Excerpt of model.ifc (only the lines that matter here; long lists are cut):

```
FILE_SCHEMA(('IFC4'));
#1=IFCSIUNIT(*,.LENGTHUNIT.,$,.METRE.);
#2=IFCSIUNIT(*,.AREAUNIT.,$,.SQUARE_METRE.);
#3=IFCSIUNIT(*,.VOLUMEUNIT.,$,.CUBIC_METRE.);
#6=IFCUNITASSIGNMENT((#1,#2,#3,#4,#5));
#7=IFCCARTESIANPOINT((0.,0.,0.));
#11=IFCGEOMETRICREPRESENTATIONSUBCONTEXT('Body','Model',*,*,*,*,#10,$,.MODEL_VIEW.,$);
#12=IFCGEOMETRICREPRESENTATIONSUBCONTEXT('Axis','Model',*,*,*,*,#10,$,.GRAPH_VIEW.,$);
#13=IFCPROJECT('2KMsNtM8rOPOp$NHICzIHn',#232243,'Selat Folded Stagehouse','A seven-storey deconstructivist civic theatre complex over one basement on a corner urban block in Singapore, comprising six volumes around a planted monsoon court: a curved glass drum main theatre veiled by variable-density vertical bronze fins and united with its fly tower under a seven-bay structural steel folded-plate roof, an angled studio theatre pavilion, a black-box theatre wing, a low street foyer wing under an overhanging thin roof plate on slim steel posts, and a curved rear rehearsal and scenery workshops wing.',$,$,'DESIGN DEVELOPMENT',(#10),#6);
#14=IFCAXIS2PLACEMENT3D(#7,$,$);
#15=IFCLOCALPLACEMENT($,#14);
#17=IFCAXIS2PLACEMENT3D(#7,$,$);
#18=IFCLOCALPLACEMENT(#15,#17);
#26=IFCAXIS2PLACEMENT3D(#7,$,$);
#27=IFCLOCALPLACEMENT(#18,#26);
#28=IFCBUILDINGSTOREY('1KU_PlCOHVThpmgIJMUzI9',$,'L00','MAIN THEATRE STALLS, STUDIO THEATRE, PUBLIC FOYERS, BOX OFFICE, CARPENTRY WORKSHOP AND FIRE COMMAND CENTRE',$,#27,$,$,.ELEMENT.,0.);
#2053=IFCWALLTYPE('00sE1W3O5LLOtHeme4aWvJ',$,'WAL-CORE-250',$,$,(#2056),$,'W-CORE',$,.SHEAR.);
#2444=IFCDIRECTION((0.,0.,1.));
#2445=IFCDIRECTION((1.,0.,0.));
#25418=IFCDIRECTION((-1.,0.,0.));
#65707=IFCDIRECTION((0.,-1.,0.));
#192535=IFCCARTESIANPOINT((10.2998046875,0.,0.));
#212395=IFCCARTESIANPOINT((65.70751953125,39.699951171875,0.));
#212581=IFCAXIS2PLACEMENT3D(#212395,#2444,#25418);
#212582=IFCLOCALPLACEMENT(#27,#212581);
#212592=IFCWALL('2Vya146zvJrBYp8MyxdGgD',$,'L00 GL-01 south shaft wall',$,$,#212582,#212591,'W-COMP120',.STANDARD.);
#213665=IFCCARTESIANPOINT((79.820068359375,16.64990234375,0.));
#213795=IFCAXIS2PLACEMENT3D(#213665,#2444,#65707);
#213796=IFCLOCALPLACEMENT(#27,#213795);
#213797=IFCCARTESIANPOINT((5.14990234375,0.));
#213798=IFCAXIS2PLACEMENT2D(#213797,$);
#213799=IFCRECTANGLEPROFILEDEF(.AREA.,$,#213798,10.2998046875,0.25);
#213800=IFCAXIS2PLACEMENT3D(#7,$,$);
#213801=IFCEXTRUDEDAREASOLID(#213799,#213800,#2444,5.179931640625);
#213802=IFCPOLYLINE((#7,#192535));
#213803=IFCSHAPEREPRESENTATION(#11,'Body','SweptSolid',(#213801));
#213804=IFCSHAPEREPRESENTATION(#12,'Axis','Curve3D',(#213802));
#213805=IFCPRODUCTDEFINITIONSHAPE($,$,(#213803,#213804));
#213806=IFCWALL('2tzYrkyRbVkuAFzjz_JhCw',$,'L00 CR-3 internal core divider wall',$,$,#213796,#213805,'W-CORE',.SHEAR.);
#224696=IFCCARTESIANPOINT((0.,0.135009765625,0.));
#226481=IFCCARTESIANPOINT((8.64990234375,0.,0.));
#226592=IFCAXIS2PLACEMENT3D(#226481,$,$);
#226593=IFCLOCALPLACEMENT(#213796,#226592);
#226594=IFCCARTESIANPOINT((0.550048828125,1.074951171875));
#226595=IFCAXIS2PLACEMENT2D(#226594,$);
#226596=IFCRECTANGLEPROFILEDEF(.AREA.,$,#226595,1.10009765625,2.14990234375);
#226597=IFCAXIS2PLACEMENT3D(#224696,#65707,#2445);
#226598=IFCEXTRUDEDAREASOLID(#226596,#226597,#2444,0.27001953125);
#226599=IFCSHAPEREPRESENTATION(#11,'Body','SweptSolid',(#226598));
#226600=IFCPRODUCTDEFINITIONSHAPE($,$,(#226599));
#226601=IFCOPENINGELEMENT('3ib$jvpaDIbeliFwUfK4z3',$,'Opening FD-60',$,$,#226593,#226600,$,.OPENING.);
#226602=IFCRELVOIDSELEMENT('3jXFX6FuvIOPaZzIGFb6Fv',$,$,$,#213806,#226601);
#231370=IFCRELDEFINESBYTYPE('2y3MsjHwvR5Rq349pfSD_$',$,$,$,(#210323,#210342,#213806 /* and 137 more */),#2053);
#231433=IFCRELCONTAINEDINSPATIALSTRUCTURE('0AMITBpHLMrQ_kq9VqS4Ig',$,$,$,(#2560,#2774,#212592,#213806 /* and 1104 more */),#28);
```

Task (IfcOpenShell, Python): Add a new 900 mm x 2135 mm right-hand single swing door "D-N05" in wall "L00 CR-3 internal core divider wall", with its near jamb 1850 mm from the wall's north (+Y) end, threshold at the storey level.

```python
import numpy as np
import ifcopenshell
import ifcopenshell.api.feature
import ifcopenshell.api.geometry
import ifcopenshell.api.root
import ifcopenshell.api.spatial
import ifcopenshell.geom
import ifcopenshell.util.element
import ifcopenshell.util.placement
import ifcopenshell.util.representation
import ifcopenshell.util.shape
import ifcopenshell.util.unit

model = ifcopenshell.open("model.ifc")
unit_scale = ifcopenshell.util.unit.calculate_unit_scale(model)
settings = ifcopenshell.geom.settings()


def volume(element):
    """Net volume in cubic metres, openings subtracted."""
    shape = ifcopenshell.geom.create_shape(settings, element)
    return ifcopenshell.util.shape.get_volume(shape.geometry)


wall = model.by_guid("2tzYrkyRbVkuAFzjz_JhCw")
storey = ifcopenshell.util.element.get_container(wall, ifc_class="IfcBuildingStorey")
context = ifcopenshell.util.representation.get_context(model, "Model", "Body", "MODEL_VIEW")
before = volume(wall)

width, height, from_end, sill = 0.9, 2.135, 1.85, 0.0  # metres

# The wall runs along its own X axis, and the end named is its -X end.
wall_shape = ifcopenshell.geom.create_shape(settings, wall)
x, y, z = ifcopenshell.util.shape.get_vertices(wall_shape.geometry).T
start = x.min() + from_end
face, thickness = float(y.min()), float(y.max() - y.min())
wall_matrix = ifcopenshell.util.placement.get_local_placement(wall.ObjectPlacement)
level = ifcopenshell.util.placement.get_local_placement(storey.ObjectPlacement)[2, 3]


def in_wall(x, y):
    """Placement at x, y metres in the wall's axes, at sill height."""
    matrix = wall_matrix.copy()
    matrix[:, 3] = wall_matrix @ np.array([x / unit_scale, y / unit_scale, 0.0, 1.0])
    matrix[2, 3] = level + sill / unit_scale
    return matrix


# Opening: a box that overshoots both wall faces by 50 mm.
opening = ifcopenshell.api.root.create_entity(model, ifc_class="IfcOpeningElement", predefined_type="OPENING")
box = ifcopenshell.api.geometry.add_wall_representation(
    model, context=context, length=width, height=height, thickness=thickness + 0.1
)
ifcopenshell.api.geometry.assign_representation(model, product=opening, representation=box)
ifcopenshell.api.geometry.edit_object_placement(model, product=opening, matrix=in_wall(start, face - 0.05), is_si=False)
ifcopenshell.api.feature.add_feature(model, feature=opening, element=wall)

door = ifcopenshell.api.root.create_entity(model, ifc_class="IfcDoor", name="D-N05", predefined_type="DOOR")
door.OverallWidth, door.OverallHeight = width / unit_scale, height / unit_scale
door.OperationType = "SINGLE_SWING_RIGHT"
body = ifcopenshell.api.geometry.add_door_representation(
    model,
    context=context,
    overall_width=door.OverallWidth,
    overall_height=door.OverallHeight,
    operation_type="SINGLE_SWING_RIGHT",
    lining_properties={"LiningDepth": thickness / unit_scale, "ThresholdDepth": thickness / unit_scale},
)
ifcopenshell.api.geometry.assign_representation(model, product=door, representation=body)
ifcopenshell.api.spatial.assign_container(model, products=[door], relating_structure=storey)
ifcopenshell.api.feature.add_filling(model, opening=opening, element=door)

# The lining spans the wall, so the door starts at the wall face.
ifcopenshell.api.geometry.edit_object_placement(model, product=door, matrix=in_wall(start, face), is_si=False)

after = volume(wall)

print(f"wall volume {before:.3f} -> {after:.3f} m3")

model.write("model_rev.ifc")
```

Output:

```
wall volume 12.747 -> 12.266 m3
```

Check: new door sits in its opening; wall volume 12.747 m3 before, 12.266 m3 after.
